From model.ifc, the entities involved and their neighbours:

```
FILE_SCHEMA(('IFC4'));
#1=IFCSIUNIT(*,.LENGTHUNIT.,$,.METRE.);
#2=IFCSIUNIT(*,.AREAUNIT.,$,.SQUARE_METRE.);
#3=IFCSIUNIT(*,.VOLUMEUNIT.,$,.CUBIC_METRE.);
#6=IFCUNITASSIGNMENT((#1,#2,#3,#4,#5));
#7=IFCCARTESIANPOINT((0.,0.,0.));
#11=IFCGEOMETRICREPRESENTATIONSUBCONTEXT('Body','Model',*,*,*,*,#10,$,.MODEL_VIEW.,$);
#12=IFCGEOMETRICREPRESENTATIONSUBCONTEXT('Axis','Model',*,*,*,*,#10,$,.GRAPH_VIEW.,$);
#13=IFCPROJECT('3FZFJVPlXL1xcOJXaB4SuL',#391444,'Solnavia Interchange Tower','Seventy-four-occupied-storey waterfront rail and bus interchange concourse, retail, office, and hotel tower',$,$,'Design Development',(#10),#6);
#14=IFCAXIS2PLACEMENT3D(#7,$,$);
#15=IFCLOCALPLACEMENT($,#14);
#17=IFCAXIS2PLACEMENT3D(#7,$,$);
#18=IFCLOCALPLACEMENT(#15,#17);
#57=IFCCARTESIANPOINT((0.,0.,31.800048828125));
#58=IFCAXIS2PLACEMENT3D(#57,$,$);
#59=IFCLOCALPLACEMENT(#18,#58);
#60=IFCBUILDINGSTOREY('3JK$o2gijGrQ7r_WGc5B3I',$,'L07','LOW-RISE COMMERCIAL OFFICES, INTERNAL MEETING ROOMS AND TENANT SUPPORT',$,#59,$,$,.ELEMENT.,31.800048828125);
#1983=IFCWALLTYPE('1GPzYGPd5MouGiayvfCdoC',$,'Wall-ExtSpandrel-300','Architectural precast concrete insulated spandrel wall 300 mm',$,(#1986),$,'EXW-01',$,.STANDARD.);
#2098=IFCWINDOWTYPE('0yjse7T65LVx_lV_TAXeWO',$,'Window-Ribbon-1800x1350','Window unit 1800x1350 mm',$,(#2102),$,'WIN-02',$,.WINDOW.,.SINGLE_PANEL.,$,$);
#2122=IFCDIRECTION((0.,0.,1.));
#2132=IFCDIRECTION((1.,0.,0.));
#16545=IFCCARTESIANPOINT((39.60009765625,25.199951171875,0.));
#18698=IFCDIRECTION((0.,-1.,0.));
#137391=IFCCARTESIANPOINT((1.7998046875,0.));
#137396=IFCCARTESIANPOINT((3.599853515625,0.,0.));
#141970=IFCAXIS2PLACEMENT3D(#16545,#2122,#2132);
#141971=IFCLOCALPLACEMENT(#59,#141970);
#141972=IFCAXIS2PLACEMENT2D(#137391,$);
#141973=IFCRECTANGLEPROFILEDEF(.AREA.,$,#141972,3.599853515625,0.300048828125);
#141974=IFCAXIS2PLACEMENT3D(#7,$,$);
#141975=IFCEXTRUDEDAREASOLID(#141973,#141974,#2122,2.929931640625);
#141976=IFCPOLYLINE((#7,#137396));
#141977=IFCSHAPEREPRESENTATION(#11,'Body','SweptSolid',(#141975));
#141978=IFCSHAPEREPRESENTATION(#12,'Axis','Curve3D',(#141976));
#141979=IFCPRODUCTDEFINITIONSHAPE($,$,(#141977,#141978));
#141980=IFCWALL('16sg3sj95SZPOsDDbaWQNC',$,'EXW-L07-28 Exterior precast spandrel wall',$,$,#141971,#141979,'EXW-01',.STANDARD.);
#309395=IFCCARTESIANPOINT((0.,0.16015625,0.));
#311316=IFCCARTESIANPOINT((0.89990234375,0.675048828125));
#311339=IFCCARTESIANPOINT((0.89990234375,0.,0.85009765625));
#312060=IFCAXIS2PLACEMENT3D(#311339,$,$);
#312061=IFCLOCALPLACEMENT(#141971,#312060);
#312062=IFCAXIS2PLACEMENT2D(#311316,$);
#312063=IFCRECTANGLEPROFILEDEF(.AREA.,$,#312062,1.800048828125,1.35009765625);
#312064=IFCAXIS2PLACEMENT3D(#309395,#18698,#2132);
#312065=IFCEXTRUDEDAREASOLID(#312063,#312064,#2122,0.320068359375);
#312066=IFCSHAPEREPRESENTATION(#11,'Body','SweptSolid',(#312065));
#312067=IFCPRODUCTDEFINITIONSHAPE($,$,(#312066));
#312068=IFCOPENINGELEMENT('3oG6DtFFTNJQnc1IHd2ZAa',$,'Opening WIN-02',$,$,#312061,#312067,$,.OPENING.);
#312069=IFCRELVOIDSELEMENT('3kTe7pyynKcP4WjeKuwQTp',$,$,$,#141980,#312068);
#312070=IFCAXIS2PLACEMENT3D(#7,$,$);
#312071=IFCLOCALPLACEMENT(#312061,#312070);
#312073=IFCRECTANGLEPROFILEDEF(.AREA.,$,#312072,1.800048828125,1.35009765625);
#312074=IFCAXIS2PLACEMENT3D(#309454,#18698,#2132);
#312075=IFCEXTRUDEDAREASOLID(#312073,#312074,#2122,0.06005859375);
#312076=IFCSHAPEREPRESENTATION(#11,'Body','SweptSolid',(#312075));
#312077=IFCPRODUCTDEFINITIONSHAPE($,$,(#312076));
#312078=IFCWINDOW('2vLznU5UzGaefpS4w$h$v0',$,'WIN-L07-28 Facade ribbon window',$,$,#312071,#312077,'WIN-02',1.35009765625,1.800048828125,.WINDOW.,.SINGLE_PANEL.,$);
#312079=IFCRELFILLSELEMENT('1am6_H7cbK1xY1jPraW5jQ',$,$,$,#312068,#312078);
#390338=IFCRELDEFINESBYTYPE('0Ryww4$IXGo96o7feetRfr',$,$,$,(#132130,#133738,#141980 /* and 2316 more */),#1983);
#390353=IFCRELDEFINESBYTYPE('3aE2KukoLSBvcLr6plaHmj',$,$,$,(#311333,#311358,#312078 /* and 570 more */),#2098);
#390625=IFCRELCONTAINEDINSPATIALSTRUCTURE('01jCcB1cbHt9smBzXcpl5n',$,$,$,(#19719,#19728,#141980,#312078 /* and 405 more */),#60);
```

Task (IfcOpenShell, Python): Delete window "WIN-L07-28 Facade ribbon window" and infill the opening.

```python
import ifcopenshell
import ifcopenshell.api.feature
import ifcopenshell.api.root
import ifcopenshell.geom
import ifcopenshell.util.shape

model = ifcopenshell.open("model.ifc")
settings = ifcopenshell.geom.settings()


def volume(element):
    """Net volume in cubic metres, openings subtracted."""
    shape = ifcopenshell.geom.create_shape(settings, element)
    return ifcopenshell.util.shape.get_volume(shape.geometry)


window = model.by_guid("2vLznU5UzGaefpS4w$h$v0")
opening = window.FillsVoids[0].RelatingOpeningElement
wall = opening.VoidsElements[0].RelatingBuildingElement
before = volume(wall)

ifcopenshell.api.root.remove_product(model, product=window)
ifcopenshell.api.feature.remove_feature(model, feature=opening)

after = volume(wall)

print(f"wall volume {before:.3f} -> {after:.3f} m3")

model.write("model_v2.ifc")
```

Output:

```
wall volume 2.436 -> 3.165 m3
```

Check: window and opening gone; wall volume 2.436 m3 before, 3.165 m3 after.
